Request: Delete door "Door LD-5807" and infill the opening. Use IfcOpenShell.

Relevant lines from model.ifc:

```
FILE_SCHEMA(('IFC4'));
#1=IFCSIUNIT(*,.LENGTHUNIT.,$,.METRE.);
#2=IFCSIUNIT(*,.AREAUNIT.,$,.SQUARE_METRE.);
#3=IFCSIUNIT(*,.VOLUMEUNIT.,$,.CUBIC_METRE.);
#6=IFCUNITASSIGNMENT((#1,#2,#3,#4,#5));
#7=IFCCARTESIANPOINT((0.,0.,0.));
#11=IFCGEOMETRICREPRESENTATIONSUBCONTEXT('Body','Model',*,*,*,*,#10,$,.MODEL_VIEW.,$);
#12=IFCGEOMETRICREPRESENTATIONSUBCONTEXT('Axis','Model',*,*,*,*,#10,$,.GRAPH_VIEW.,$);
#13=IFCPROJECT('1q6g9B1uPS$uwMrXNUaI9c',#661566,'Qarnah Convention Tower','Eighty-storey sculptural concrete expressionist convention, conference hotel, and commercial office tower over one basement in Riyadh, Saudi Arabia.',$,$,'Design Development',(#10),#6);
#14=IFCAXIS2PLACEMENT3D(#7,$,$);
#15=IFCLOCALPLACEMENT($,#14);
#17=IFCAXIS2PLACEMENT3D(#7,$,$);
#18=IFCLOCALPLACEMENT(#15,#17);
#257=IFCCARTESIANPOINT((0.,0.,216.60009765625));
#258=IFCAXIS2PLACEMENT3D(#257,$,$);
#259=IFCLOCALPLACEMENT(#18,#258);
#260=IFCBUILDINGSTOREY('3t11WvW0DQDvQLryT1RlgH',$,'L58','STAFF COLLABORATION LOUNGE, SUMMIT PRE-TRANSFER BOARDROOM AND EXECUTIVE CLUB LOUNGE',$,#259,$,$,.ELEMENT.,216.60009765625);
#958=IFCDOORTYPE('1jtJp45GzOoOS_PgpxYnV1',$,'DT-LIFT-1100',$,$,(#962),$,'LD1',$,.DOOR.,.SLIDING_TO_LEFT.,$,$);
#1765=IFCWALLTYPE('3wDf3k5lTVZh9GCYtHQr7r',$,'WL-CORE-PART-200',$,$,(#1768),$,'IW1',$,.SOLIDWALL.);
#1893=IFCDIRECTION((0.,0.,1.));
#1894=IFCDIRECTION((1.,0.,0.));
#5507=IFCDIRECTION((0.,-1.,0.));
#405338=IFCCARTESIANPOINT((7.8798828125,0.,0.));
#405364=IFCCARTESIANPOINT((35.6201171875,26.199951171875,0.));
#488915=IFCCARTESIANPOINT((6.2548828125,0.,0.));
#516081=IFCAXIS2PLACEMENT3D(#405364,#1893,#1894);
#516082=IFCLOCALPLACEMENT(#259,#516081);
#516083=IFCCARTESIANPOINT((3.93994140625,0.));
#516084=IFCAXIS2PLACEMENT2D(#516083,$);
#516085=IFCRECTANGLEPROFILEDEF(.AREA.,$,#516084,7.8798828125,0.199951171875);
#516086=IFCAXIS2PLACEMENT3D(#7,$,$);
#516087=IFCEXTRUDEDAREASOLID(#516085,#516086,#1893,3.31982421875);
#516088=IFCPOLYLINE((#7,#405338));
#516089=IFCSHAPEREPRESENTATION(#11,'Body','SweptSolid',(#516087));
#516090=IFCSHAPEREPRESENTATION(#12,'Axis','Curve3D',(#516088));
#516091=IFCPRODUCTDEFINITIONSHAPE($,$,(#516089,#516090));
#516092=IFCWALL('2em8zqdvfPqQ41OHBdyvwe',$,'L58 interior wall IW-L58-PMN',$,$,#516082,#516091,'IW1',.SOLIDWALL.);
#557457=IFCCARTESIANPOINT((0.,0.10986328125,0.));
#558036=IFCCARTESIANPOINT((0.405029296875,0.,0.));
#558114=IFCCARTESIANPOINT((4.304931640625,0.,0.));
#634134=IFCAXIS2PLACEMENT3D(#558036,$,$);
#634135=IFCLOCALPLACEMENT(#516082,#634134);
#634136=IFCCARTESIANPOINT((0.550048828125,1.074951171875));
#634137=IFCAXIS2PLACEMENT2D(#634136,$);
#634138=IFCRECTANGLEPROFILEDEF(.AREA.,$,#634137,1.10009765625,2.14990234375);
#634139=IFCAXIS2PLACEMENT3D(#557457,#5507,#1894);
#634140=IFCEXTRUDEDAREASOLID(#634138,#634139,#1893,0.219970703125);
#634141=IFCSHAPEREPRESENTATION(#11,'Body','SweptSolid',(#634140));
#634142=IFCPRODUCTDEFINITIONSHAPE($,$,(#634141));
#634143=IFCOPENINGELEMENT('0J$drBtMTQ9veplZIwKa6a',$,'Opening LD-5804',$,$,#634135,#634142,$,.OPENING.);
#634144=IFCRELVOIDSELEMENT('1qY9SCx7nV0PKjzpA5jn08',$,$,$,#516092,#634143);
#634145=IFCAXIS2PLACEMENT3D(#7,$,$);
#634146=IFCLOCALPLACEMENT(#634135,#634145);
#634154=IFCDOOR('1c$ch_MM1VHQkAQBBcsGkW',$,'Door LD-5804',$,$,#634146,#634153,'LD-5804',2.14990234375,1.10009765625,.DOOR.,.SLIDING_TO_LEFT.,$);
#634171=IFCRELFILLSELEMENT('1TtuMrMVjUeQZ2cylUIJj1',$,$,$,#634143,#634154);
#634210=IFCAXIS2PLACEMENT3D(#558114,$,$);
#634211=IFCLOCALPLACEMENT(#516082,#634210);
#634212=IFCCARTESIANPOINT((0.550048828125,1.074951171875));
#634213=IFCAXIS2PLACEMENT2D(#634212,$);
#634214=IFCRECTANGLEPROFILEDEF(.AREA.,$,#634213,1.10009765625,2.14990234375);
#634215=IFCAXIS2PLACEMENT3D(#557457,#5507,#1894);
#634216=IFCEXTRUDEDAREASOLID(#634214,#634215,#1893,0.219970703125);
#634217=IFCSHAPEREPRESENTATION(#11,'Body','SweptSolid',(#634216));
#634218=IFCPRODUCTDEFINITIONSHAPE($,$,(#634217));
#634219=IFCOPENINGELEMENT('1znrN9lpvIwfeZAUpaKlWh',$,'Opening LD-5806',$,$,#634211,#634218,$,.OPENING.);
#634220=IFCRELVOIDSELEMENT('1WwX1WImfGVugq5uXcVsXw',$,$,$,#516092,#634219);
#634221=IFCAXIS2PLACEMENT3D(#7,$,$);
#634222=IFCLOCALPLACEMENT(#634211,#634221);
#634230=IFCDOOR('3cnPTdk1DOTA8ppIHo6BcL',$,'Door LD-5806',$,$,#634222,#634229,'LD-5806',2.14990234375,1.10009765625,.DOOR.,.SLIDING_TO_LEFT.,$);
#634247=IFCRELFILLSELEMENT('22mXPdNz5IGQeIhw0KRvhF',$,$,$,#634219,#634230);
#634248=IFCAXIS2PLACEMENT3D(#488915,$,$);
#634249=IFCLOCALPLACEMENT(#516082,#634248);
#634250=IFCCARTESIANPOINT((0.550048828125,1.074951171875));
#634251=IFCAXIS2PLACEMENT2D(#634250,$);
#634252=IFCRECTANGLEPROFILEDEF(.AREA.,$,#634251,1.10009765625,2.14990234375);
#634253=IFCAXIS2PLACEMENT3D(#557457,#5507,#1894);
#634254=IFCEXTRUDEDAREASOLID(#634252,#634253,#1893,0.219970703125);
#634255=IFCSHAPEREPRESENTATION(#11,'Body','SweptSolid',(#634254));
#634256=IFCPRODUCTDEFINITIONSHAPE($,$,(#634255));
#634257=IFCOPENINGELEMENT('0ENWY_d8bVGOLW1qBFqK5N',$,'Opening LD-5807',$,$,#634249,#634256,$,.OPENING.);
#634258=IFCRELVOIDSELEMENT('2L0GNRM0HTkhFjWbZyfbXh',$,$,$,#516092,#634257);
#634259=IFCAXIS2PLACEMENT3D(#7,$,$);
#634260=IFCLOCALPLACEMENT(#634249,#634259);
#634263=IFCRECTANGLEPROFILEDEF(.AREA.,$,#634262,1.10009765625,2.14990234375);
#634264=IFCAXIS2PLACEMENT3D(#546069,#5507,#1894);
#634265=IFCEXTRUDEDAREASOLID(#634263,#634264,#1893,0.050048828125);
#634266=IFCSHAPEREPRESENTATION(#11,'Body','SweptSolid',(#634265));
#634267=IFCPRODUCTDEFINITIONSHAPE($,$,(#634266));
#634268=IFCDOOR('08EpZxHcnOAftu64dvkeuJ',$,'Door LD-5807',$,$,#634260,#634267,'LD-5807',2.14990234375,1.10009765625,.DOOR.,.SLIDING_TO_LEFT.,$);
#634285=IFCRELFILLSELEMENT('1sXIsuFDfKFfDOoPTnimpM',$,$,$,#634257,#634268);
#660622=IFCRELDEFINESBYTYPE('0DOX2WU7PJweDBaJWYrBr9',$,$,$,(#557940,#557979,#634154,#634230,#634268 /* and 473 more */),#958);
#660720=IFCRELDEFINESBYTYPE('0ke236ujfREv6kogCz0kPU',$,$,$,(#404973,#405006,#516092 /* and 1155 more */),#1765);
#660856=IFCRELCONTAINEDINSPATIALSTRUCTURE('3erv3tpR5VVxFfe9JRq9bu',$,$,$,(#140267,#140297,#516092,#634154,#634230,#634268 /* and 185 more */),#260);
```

```python
import ifcopenshell
import ifcopenshell.api.feature
import ifcopenshell.api.root
import ifcopenshell.geom
import ifcopenshell.util.shape

model = ifcopenshell.open("model.ifc")
settings = ifcopenshell.geom.settings()


def volume(element):
    """Net volume in cubic metres, openings subtracted."""
    shape = ifcopenshell.geom.create_shape(settings, element)
    return ifcopenshell.util.shape.get_volume(shape.geometry)


door = model.by_guid("08EpZxHcnOAftu64dvkeuJ")
opening = door.FillsVoids[0].RelatingOpeningElement
wall = opening.VoidsElements[0].RelatingBuildingElement
before = volume(wall)

ifcopenshell.api.root.remove_product(model, product=door)
ifcopenshell.api.feature.remove_feature(model, feature=opening)

after = volume(wall)

print(f"wall volume {before:.3f} -> {after:.3f} m3")

model.write("model_rev.ifc")
```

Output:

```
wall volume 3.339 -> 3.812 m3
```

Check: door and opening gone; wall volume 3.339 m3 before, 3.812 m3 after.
